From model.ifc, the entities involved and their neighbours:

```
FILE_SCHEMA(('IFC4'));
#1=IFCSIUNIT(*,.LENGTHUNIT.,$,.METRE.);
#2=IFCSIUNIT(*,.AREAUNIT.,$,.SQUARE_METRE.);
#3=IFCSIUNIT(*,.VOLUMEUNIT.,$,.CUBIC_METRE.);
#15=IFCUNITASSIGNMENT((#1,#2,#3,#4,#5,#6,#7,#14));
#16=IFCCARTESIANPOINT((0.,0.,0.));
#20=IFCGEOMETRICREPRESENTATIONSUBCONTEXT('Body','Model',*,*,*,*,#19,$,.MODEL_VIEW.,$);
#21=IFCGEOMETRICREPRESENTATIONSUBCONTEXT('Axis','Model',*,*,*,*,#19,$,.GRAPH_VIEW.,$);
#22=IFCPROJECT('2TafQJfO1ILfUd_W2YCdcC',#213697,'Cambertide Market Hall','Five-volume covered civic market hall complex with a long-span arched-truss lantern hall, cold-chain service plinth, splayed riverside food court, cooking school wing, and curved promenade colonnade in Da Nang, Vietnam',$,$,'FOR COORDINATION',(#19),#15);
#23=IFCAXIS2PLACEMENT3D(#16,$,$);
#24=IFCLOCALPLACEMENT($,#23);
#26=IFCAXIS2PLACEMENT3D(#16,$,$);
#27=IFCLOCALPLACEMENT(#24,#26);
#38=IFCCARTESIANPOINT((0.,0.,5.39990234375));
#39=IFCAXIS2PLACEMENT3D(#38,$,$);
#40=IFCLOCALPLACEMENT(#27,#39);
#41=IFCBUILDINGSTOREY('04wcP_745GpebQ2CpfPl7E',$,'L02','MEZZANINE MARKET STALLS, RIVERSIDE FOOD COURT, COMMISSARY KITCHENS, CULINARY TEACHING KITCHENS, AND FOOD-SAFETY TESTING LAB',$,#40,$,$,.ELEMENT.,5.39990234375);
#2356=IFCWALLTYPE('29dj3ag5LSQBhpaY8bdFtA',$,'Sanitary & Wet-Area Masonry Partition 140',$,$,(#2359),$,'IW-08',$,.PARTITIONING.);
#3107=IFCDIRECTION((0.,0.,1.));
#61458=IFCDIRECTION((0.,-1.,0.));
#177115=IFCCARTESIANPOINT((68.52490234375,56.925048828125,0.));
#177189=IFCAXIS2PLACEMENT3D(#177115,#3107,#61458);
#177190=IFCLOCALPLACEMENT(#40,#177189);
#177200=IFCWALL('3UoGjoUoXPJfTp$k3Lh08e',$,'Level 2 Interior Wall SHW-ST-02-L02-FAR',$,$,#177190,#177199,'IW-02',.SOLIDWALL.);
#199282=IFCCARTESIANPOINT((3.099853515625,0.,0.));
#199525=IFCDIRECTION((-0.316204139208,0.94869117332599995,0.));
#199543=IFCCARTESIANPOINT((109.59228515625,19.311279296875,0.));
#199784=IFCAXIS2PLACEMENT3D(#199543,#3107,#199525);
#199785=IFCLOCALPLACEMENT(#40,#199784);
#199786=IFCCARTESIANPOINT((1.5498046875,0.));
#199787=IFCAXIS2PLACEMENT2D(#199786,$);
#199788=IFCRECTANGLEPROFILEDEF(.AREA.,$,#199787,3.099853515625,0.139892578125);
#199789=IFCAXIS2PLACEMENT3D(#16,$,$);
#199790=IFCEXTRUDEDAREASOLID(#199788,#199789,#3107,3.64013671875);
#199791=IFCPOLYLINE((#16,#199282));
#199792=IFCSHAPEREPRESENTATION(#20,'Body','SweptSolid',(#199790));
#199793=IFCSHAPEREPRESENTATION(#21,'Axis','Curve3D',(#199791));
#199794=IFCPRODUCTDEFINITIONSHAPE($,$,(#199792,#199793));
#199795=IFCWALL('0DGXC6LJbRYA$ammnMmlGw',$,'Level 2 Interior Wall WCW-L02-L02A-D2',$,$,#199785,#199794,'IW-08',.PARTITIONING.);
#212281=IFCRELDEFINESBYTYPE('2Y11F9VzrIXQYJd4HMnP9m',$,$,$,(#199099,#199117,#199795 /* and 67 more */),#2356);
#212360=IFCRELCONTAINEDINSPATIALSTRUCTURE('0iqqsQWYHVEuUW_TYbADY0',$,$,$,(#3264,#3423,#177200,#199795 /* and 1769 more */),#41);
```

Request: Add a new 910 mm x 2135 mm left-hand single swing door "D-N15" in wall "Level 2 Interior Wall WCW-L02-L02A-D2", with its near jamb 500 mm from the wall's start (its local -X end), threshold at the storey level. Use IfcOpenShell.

```python
import numpy as np
import ifcopenshell
import ifcopenshell.api.feature
import ifcopenshell.api.geometry
import ifcopenshell.api.root
import ifcopenshell.api.spatial
import ifcopenshell.geom
import ifcopenshell.util.element
import ifcopenshell.util.placement
import ifcopenshell.util.representation
import ifcopenshell.util.shape
import ifcopenshell.util.unit

model = ifcopenshell.open("model.ifc")
unit_scale = ifcopenshell.util.unit.calculate_unit_scale(model)
settings = ifcopenshell.geom.settings()


def volume(element):
    """Net volume in cubic metres, openings subtracted."""
    shape = ifcopenshell.geom.create_shape(settings, element)
    return ifcopenshell.util.shape.get_volume(shape.geometry)


wall = model.by_id(199795)
storey = ifcopenshell.util.element.get_container(wall, ifc_class="IfcBuildingStorey")
context = ifcopenshell.util.representation.get_context(model, "Model", "Body", "MODEL_VIEW")
before = volume(wall)

width, height, from_end, sill = 0.91, 2.135, 0.5, 0.0  # metres

# The wall runs along its own X axis, and the end named is its -X end.
wall_shape = ifcopenshell.geom.create_shape(settings, wall)
x, y, z = ifcopenshell.util.shape.get_vertices(wall_shape.geometry).T
start = x.min() + from_end
face, thickness = float(y.min()), float(y.max() - y.min())
wall_matrix = ifcopenshell.util.placement.get_local_placement(wall.ObjectPlacement)
level = ifcopenshell.util.placement.get_local_placement(storey.ObjectPlacement)[2, 3]


def in_wall(x, y):
    """Placement at x, y metres in the wall's axes, at sill height."""
    matrix = wall_matrix.copy()
    matrix[:, 3] = wall_matrix @ np.array([x / unit_scale, y / unit_scale, 0.0, 1.0])
    matrix[2, 3] = level + sill / unit_scale
    return matrix


# Opening: a box that overshoots both wall faces by 50 mm.
opening = ifcopenshell.api.root.create_entity(model, ifc_class="IfcOpeningElement", predefined_type="OPENING")
box = ifcopenshell.api.geometry.add_wall_representation(
    model, context=context, length=width, height=height, thickness=thickness + 0.1
)
ifcopenshell.api.geometry.assign_representation(model, product=opening, representation=box)
ifcopenshell.api.geometry.edit_object_placement(model, product=opening, matrix=in_wall(start, face - 0.05), is_si=False)
ifcopenshell.api.feature.add_feature(model, feature=opening, element=wall)

door = ifcopenshell.api.root.create_entity(model, ifc_class="IfcDoor", name="D-N15", predefined_type="DOOR")
door.OverallWidth, door.OverallHeight = width / unit_scale, height / unit_scale
door.OperationType = "SINGLE_SWING_LEFT"
body = ifcopenshell.api.geometry.add_door_representation(
    model,
    context=context,
    overall_width=door.OverallWidth,
    overall_height=door.OverallHeight,
    operation_type="SINGLE_SWING_LEFT",
    lining_properties={"LiningDepth": thickness / unit_scale, "ThresholdDepth": thickness / unit_scale},
)
ifcopenshell.api.geometry.assign_representation(model, product=door, representation=body)
ifcopenshell.api.spatial.assign_container(model, products=[door], relating_structure=storey)
ifcopenshell.api.feature.add_filling(model, opening=opening, element=door)

# The lining spans the wall, so the door starts at the wall face.
ifcopenshell.api.geometry.edit_object_placement(model, product=door, matrix=in_wall(start, face), is_si=False)

after = volume(wall)

print(f"wall volume {before:.3f} -> {after:.3f} m3")

model.write("model-out.ifc")
```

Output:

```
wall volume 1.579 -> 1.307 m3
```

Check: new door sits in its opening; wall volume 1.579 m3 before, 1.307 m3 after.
